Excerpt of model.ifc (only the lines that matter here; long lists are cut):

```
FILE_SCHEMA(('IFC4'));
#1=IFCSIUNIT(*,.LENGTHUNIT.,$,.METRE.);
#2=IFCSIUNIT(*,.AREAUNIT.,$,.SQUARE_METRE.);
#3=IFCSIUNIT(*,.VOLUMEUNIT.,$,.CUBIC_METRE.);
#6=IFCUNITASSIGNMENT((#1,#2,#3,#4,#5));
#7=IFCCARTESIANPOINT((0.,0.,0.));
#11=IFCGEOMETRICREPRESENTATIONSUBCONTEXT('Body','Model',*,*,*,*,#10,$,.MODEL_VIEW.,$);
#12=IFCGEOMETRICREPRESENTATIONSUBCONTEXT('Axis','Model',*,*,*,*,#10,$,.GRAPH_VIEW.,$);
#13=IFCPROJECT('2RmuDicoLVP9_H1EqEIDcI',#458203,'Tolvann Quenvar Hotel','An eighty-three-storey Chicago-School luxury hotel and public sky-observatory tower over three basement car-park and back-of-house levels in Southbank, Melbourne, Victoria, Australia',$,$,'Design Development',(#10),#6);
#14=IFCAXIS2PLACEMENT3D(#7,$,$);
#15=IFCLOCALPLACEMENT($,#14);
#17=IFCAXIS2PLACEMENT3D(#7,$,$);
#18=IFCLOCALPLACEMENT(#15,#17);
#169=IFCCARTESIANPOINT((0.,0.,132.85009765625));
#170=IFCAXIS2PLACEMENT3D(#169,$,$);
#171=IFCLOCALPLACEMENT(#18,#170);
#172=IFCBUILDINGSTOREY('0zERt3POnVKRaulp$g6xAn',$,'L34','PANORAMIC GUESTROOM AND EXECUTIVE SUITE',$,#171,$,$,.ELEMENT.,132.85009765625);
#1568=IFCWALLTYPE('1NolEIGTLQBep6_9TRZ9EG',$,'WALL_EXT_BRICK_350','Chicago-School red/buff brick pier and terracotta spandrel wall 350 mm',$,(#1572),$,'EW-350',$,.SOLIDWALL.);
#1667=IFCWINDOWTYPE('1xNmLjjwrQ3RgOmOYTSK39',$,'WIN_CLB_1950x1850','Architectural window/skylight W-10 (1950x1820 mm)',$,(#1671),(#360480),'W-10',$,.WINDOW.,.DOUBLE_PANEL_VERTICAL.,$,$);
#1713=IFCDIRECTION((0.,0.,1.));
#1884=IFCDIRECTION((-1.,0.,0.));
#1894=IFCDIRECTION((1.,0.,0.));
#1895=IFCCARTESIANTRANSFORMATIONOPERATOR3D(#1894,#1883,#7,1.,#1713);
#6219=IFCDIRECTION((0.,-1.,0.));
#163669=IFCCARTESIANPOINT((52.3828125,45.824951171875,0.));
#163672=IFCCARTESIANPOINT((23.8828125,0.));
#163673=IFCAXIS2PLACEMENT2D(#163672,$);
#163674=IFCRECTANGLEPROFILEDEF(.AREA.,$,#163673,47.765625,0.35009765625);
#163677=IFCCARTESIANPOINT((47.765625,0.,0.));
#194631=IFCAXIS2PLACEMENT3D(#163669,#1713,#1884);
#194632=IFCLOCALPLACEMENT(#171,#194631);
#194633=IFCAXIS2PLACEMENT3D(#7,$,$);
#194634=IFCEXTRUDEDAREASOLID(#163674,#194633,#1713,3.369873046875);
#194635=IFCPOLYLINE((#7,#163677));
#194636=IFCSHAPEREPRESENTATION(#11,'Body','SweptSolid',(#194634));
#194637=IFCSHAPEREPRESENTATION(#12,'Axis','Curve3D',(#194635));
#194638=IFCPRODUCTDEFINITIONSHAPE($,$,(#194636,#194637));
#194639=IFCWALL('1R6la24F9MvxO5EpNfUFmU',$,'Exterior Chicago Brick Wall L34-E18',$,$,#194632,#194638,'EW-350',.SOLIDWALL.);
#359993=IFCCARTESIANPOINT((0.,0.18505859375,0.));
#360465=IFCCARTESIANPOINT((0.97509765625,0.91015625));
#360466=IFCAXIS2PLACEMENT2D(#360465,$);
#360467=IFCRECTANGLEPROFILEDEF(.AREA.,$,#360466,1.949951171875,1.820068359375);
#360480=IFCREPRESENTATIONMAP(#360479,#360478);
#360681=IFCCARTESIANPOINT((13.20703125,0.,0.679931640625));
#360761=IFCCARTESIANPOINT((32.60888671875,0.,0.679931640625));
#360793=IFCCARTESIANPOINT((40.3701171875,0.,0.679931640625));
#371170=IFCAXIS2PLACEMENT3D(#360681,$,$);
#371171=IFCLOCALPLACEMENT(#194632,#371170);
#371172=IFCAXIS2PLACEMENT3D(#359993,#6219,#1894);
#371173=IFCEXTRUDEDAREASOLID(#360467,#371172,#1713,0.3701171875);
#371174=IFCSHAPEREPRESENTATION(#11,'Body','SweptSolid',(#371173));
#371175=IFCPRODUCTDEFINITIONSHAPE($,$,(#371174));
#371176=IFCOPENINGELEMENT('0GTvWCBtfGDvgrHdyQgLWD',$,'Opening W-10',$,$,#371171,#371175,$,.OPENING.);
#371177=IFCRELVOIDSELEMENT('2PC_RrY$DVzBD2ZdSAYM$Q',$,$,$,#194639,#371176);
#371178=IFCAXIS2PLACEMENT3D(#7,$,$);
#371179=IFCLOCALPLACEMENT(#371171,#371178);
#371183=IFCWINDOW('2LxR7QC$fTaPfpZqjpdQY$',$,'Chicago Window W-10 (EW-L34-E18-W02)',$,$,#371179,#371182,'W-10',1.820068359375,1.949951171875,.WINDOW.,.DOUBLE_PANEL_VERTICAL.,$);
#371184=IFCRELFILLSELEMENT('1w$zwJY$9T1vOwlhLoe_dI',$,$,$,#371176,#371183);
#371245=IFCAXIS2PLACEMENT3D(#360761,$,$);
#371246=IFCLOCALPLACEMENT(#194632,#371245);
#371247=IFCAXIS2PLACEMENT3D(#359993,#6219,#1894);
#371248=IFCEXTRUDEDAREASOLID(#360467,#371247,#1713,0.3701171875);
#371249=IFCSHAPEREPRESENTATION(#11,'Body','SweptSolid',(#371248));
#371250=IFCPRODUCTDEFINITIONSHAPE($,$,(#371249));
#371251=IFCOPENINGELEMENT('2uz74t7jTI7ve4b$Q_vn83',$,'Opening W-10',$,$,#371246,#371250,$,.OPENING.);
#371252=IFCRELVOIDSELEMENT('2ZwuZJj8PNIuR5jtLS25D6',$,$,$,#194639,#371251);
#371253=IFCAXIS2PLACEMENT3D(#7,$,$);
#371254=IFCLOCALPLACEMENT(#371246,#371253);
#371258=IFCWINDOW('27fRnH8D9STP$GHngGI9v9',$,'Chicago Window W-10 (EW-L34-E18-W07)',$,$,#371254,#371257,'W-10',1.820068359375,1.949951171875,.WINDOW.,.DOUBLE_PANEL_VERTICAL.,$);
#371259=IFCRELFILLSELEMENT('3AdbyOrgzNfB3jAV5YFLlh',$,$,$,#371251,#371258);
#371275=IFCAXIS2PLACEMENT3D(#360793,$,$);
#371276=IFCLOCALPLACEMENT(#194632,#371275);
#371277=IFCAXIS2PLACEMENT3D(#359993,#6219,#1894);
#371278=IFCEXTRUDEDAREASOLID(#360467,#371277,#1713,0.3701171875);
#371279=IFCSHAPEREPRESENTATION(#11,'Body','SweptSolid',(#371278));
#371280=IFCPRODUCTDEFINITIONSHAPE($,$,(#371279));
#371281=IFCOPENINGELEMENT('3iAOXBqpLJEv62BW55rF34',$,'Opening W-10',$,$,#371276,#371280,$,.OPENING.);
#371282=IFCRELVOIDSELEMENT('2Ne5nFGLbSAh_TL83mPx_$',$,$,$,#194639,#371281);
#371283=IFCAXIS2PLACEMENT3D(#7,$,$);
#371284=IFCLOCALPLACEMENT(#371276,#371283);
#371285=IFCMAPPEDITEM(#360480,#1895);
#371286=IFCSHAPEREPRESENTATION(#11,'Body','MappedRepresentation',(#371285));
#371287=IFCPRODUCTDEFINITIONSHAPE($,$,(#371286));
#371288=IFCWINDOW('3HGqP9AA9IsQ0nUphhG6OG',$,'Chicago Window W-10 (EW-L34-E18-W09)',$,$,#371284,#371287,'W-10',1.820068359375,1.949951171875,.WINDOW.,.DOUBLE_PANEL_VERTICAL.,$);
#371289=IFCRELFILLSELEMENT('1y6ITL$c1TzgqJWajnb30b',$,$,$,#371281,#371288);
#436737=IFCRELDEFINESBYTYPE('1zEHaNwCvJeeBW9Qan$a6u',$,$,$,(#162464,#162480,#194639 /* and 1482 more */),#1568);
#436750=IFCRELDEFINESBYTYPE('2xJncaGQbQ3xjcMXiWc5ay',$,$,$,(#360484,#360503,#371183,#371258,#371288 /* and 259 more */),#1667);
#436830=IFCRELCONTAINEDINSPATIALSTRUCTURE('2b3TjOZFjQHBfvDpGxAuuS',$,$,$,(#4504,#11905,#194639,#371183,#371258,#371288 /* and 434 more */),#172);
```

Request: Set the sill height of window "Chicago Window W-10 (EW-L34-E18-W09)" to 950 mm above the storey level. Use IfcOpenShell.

```python
import numpy as np
import ifcopenshell
import ifcopenshell.api.geometry
import ifcopenshell.geom
import ifcopenshell.util.element
import ifcopenshell.util.placement
import ifcopenshell.util.shape
import ifcopenshell.util.unit

model = ifcopenshell.open("model.ifc")
unit_scale = ifcopenshell.util.unit.calculate_unit_scale(model)

window = model.by_id(371288)
opening = window.FillsVoids[0].RelatingOpeningElement
storey = ifcopenshell.util.element.get_container(window, ifc_class="IfcBuildingStorey")
level = ifcopenshell.util.placement.get_local_placement(storey.ObjectPlacement)[2, 3]

# The opening's origin need not be at the sill, so measure its lowest point.
shape = ifcopenshell.geom.create_shape(ifcopenshell.geom.settings(), opening)
bottom = ifcopenshell.util.shape.get_shape_bottom_elevation(shape, shape.geometry) / unit_scale
dz = level + 0.95 / unit_scale - bottom

shift = np.array([0.0, 0.0, dz])
# The window is placed relative to its opening, so it follows when the opening moves.
matrix = ifcopenshell.util.placement.get_local_placement(opening.ObjectPlacement)
matrix[:3, 3] += shift
ifcopenshell.api.geometry.edit_object_placement(
    model, product=opening, matrix=matrix, is_si=False, should_transform_children=True
)

print(f"moved by {dz * unit_scale:+.3f} m")

model.write("model_v2.ifc")
```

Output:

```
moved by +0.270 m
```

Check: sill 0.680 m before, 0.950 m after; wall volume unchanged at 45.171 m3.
